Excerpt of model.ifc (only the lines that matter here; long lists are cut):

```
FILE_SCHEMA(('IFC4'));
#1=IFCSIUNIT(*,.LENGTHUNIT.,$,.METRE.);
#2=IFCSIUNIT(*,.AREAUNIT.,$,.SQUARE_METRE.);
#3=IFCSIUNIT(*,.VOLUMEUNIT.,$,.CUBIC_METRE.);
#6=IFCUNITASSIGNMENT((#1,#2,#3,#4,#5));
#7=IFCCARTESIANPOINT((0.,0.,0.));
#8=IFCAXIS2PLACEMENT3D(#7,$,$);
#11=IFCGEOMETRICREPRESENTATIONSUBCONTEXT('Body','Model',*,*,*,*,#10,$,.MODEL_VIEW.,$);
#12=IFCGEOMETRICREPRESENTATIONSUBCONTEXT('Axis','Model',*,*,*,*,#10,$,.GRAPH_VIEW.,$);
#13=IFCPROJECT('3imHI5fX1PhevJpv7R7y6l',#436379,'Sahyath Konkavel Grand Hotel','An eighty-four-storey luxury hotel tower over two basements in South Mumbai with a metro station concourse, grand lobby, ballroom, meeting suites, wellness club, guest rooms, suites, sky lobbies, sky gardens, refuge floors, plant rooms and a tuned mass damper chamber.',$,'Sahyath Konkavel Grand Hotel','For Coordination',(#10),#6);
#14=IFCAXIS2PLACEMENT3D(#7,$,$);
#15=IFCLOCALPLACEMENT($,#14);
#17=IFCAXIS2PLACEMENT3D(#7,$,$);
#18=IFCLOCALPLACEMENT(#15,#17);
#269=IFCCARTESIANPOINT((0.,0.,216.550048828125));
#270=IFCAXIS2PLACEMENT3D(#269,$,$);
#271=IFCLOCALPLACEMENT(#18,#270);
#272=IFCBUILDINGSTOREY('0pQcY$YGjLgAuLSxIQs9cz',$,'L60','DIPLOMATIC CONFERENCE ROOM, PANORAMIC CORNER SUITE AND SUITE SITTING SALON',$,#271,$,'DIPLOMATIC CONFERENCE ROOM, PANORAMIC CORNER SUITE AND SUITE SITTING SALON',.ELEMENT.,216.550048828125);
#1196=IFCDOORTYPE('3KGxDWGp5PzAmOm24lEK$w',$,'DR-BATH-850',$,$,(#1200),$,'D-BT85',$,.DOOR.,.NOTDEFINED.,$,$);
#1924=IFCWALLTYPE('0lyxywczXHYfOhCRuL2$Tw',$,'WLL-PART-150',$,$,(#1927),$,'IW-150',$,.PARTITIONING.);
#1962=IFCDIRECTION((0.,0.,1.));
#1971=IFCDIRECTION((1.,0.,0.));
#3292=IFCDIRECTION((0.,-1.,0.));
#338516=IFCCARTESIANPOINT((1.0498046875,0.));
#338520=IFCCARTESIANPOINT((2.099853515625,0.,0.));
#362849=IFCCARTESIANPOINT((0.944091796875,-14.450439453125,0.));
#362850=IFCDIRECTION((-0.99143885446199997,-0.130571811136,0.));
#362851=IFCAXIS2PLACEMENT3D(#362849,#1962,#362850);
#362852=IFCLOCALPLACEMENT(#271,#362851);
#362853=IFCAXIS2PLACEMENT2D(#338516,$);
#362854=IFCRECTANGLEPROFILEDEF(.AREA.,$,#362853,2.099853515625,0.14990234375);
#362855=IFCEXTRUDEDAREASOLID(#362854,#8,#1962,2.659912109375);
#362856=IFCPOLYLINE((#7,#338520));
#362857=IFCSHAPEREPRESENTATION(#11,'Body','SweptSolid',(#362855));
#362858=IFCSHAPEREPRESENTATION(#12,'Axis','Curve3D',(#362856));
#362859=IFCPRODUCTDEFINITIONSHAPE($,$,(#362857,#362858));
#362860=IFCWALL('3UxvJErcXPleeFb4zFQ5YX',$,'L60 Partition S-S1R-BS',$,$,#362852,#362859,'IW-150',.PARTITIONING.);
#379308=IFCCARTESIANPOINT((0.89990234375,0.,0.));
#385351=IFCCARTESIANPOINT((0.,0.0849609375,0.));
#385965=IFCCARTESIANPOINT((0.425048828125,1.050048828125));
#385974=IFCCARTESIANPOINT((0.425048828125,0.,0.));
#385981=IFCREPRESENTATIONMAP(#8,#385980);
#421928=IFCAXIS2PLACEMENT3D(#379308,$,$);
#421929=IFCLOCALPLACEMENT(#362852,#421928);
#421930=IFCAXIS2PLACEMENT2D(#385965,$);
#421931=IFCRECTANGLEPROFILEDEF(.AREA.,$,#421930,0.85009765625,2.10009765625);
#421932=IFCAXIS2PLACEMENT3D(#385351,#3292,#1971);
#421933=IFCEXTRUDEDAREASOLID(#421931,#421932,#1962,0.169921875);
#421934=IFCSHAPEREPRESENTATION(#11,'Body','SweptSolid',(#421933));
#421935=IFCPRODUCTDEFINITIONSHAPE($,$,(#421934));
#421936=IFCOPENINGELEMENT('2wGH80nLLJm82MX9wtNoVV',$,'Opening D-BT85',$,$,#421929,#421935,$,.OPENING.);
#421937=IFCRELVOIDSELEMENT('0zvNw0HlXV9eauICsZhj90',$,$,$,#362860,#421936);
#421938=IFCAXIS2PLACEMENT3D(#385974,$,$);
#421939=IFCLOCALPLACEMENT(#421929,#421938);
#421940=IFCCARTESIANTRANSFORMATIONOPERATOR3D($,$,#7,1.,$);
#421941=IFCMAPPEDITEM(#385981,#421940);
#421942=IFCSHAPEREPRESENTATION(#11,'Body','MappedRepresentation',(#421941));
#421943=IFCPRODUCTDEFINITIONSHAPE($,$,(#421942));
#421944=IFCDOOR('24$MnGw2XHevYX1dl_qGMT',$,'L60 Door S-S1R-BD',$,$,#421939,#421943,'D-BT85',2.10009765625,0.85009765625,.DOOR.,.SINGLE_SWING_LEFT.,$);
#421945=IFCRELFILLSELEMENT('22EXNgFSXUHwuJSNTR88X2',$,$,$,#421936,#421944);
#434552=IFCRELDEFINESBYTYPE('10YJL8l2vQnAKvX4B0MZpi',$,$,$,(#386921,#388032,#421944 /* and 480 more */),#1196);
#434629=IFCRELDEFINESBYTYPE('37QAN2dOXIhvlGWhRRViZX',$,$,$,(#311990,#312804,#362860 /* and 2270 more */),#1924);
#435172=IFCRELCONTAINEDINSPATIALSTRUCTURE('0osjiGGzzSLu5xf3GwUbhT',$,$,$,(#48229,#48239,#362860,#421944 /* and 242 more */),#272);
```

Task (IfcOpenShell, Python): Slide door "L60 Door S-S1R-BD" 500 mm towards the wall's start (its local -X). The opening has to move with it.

```python
import ifcopenshell
import ifcopenshell.api.geometry
import ifcopenshell.util.placement

model = ifcopenshell.open("model.ifc")

door = model.by_id(421944)
opening = door.FillsVoids[0].RelatingOpeningElement
wall = opening.VoidsElements[0].RelatingBuildingElement

wall_matrix = ifcopenshell.util.placement.get_local_placement(wall.ObjectPlacement)
shift = wall_matrix[:3, 0] * -0.5
before = ifcopenshell.util.placement.get_local_placement(door.ObjectPlacement)[:3, 3].copy()

# The door is placed relative to its opening, so it follows when the opening moves.
matrix = ifcopenshell.util.placement.get_local_placement(opening.ObjectPlacement)
matrix[:3, 3] += shift
ifcopenshell.api.geometry.edit_object_placement(
    model, product=opening, matrix=matrix, is_si=False, should_transform_children=True
)

after = ifcopenshell.util.placement.get_local_placement(door.ObjectPlacement)[:3, 3]
print("door moved by", (after - before).round(3) + 0.0)

model.write("model-out.ifc")
```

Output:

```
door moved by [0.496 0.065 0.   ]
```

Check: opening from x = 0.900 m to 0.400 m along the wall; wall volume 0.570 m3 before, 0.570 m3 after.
